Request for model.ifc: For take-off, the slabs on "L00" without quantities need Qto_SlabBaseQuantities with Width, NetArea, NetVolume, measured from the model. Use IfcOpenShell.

First a look at what the model holds.

```python
import ifcopenshell
import ifcopenshell.util.element
import ifcopenshell.util.unit

model = ifcopenshell.open("model.ifc")
print(model.schema)
for unit_type in ("LENGTHUNIT", "AREAUNIT", "VOLUMEUNIT"):
    print(unit_type, ifcopenshell.util.unit.calculate_unit_scale(model, unit_type))
storey = next(s for s in model.by_type("IfcBuildingStorey") if s.Name == "L00")
slabs = [e for e in ifcopenshell.util.element.get_decomposition(storey) if e.is_a("IfcSlab")]
for e in sorted(slabs, key=lambda e: e.id()):
    print(e.id(), e.is_a(), e.Name, list(ifcopenshell.util.element.get_psets(e, qtos_only=True)), sep=" | ")
```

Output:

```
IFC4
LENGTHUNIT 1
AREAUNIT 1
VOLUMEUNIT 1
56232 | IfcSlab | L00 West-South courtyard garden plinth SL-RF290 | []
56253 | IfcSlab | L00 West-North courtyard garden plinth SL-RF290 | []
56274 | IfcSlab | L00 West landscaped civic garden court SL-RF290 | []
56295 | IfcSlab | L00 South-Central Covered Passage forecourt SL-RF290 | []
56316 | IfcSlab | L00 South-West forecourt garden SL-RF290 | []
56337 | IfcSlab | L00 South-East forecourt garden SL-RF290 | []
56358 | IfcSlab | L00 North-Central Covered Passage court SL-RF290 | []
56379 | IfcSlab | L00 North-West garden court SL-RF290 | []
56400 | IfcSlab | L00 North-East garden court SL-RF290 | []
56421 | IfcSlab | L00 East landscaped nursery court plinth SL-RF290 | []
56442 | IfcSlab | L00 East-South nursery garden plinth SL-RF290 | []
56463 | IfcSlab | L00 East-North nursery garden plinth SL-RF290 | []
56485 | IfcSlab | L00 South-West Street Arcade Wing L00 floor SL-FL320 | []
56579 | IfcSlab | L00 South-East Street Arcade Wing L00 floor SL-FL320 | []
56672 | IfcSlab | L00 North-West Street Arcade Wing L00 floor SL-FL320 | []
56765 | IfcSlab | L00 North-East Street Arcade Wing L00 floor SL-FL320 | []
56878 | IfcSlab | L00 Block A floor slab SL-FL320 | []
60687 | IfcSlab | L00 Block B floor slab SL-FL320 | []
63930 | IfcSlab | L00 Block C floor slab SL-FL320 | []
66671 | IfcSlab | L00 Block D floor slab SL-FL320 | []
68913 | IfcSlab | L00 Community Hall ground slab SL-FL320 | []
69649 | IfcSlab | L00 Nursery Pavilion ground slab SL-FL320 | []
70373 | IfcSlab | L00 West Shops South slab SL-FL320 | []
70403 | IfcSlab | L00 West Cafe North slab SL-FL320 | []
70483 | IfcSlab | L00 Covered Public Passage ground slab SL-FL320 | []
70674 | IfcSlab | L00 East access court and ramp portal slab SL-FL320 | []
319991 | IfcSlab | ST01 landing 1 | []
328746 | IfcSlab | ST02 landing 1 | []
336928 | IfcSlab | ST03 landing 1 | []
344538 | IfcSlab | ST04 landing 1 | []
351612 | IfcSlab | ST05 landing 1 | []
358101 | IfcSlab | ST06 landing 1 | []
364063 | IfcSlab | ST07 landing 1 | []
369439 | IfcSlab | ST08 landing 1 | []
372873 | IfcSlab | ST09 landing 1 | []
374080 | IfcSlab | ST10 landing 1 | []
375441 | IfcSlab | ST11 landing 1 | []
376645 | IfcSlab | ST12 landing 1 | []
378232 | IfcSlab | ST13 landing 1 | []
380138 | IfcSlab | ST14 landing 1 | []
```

```python
import ifcopenshell
import ifcopenshell.api.pset
import ifcopenshell.geom
import ifcopenshell.util.element
import ifcopenshell.util.shape
import ifcopenshell.util.unit

model = ifcopenshell.open("model.ifc")
unit_scale = ifcopenshell.util.unit.calculate_unit_scale(model)
area_scale = ifcopenshell.util.unit.calculate_unit_scale(model, "AREAUNIT")
volume_scale = ifcopenshell.util.unit.calculate_unit_scale(model, "VOLUMEUNIT")
settings = ifcopenshell.geom.settings()

storey = next(s for s in model.by_type("IfcBuildingStorey") if s.Name == "L00")
slabs = [e for e in ifcopenshell.util.element.get_decomposition(storey) if e.is_a("IfcSlab")]

for e in sorted(slabs, key=lambda e: e.id()):
    if ifcopenshell.util.element.get_psets(e, qtos_only=True, should_inherit=False):
        continue
    # Geometry comes back in metres, in the element's own axes.
    shape = ifcopenshell.geom.create_shape(settings, e)
    values = {
        "Width": ifcopenshell.util.shape.get_z(shape.geometry) / unit_scale,
        "NetArea": ifcopenshell.util.shape.get_footprint_area(shape.geometry) / area_scale,
        "NetVolume": ifcopenshell.util.shape.get_volume(shape.geometry) / volume_scale,
    }
    qto = ifcopenshell.api.pset.add_qto(model, product=e, name="Qto_SlabBaseQuantities")
    ifcopenshell.api.pset.edit_qto(model, qto=qto, properties=values)
    print(e.id(), {k: round(v, 3) for k, v in values.items()})

model.write("model_edited.ifc")
```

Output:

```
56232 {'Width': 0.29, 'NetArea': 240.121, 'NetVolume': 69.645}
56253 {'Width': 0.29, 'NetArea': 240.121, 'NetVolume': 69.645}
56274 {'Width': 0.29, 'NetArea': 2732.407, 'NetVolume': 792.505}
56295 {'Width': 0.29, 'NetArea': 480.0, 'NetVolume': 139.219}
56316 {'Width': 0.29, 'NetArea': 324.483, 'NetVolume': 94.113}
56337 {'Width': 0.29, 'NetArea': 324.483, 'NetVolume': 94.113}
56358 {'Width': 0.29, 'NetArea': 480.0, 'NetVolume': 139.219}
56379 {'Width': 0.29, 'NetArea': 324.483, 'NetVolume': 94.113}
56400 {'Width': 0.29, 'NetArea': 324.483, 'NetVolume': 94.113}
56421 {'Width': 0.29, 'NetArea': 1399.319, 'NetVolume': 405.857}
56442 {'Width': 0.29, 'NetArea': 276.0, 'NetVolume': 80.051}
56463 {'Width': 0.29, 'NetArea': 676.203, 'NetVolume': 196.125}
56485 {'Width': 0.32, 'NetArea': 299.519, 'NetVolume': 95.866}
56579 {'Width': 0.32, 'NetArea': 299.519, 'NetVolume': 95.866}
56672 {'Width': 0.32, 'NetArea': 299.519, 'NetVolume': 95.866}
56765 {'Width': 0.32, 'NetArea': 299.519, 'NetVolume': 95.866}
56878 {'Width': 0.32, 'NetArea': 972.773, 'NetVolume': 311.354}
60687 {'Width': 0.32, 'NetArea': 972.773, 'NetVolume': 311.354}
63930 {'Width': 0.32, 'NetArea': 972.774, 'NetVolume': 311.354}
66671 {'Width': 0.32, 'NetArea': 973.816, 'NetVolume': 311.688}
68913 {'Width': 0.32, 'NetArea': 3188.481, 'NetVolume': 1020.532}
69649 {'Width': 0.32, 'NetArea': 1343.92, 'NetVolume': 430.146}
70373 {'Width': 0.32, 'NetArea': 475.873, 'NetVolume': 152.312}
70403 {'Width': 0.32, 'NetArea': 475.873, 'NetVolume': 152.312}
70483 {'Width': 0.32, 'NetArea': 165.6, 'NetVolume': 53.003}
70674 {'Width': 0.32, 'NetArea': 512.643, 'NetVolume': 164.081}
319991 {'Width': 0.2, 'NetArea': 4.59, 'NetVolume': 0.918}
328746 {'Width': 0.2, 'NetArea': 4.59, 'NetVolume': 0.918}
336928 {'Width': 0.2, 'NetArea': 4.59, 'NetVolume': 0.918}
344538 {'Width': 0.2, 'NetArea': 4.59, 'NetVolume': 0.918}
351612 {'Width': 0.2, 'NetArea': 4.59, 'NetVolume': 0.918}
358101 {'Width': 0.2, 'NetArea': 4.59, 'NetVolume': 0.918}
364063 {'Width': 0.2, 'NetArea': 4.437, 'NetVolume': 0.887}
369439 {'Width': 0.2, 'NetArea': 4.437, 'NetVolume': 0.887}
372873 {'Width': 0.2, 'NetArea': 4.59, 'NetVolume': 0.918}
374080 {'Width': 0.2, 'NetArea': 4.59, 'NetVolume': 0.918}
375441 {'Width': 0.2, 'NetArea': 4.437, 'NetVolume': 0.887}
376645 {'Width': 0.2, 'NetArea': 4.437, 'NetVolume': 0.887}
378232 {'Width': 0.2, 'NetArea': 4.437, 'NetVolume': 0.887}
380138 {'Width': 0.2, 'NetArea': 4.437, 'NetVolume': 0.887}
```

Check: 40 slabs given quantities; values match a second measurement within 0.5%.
